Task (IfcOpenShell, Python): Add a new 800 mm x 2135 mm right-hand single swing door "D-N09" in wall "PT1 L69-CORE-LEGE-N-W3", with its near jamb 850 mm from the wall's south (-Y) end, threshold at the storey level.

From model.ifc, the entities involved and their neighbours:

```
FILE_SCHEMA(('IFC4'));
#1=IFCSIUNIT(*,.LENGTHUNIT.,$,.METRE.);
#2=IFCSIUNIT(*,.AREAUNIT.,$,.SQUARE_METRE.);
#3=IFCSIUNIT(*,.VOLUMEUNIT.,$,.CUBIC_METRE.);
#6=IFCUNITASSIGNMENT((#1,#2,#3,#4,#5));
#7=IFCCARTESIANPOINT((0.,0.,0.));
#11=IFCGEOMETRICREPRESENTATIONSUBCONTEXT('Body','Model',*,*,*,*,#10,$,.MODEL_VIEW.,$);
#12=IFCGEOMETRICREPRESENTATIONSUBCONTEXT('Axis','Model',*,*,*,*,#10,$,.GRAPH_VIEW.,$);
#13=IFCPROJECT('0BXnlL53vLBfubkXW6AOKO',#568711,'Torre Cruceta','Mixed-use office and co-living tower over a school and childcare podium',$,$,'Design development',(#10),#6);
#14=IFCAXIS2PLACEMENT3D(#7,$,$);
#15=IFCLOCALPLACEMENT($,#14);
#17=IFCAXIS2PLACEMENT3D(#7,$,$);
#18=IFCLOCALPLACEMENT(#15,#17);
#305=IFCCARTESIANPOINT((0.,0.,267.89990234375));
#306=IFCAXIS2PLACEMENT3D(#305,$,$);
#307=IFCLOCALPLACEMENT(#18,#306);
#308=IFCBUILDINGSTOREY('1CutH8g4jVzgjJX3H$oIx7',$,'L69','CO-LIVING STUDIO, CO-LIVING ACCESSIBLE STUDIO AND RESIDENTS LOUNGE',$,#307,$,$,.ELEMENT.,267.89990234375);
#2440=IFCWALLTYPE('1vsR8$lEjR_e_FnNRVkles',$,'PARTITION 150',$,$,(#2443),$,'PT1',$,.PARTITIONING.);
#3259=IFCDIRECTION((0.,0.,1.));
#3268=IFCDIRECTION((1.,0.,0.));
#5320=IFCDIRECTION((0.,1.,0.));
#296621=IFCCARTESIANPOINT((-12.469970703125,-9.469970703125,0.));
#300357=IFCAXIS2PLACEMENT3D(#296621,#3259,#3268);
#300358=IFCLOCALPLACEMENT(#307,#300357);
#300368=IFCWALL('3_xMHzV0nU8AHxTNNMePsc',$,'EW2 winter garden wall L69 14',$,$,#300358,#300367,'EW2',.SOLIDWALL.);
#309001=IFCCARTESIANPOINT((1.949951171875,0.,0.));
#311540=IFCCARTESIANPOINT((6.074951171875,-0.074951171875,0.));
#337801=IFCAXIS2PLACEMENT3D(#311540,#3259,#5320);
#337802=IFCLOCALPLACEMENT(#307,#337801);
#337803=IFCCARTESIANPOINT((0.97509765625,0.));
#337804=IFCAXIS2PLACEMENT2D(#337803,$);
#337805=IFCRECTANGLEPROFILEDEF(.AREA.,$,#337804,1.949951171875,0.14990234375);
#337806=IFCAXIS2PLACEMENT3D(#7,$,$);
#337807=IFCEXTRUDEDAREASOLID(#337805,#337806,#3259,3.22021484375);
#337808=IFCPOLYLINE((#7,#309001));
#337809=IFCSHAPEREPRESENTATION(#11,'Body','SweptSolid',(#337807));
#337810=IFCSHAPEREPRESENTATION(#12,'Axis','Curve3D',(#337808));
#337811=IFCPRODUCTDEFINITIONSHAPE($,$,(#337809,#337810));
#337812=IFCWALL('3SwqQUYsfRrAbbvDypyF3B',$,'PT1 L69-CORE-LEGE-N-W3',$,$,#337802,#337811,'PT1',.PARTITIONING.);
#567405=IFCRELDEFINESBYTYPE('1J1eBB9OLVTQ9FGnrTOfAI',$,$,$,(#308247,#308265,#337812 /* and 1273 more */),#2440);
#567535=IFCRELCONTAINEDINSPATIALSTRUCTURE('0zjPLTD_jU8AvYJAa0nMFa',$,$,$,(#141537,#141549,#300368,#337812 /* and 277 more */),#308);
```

```python
import numpy as np
import ifcopenshell
import ifcopenshell.api.feature
import ifcopenshell.api.geometry
import ifcopenshell.api.root
import ifcopenshell.api.spatial
import ifcopenshell.geom
import ifcopenshell.util.element
import ifcopenshell.util.placement
import ifcopenshell.util.representation
import ifcopenshell.util.shape
import ifcopenshell.util.unit

model = ifcopenshell.open("model.ifc")
unit_scale = ifcopenshell.util.unit.calculate_unit_scale(model)
settings = ifcopenshell.geom.settings()


def volume(element):
    """Net volume in cubic metres, openings subtracted."""
    shape = ifcopenshell.geom.create_shape(settings, element)
    return ifcopenshell.util.shape.get_volume(shape.geometry)


wall = model.by_guid("3SwqQUYsfRrAbbvDypyF3B")
storey = ifcopenshell.util.element.get_container(wall, ifc_class="IfcBuildingStorey")
context = ifcopenshell.util.representation.get_context(model, "Model", "Body", "MODEL_VIEW")
before = volume(wall)

width, height, from_end, sill = 0.8, 2.135, 0.85, 0.0  # metres

# The wall runs along its own X axis, and the end named is its -X end.
wall_shape = ifcopenshell.geom.create_shape(settings, wall)
x, y, z = ifcopenshell.util.shape.get_vertices(wall_shape.geometry).T
start = x.min() + from_end
face, thickness = float(y.min()), float(y.max() - y.min())
wall_matrix = ifcopenshell.util.placement.get_local_placement(wall.ObjectPlacement)
level = ifcopenshell.util.placement.get_local_placement(storey.ObjectPlacement)[2, 3]


def in_wall(x, y):
    """Placement at x, y metres in the wall's axes, at sill height."""
    matrix = wall_matrix.copy()
    matrix[:, 3] = wall_matrix @ np.array([x / unit_scale, y / unit_scale, 0.0, 1.0])
    matrix[2, 3] = level + sill / unit_scale
    return matrix


# Opening: a box that overshoots both wall faces by 50 mm.
opening = ifcopenshell.api.root.create_entity(model, ifc_class="IfcOpeningElement", predefined_type="OPENING")
box = ifcopenshell.api.geometry.add_wall_representation(
    model, context=context, length=width, height=height, thickness=thickness + 0.1
)
ifcopenshell.api.geometry.assign_representation(model, product=opening, representation=box)
ifcopenshell.api.geometry.edit_object_placement(model, product=opening, matrix=in_wall(start, face - 0.05), is_si=False)
ifcopenshell.api.feature.add_feature(model, feature=opening, element=wall)

door = ifcopenshell.api.root.create_entity(model, ifc_class="IfcDoor", name="D-N09", predefined_type="DOOR")
door.OverallWidth, door.OverallHeight = width / unit_scale, height / unit_scale
door.OperationType = "SINGLE_SWING_RIGHT"
body = ifcopenshell.api.geometry.add_door_representation(
    model,
    context=context,
    overall_width=door.OverallWidth,
    overall_height=door.OverallHeight,
    operation_type="SINGLE_SWING_RIGHT",
    lining_properties={"LiningDepth": thickness / unit_scale, "ThresholdDepth": thickness / unit_scale},
)
ifcopenshell.api.geometry.assign_representation(model, product=door, representation=body)
ifcopenshell.api.spatial.assign_container(model, products=[door], relating_structure=storey)
ifcopenshell.api.feature.add_filling(model, opening=opening, element=door)

# The lining spans the wall, so the door starts at the wall face.
ifcopenshell.api.geometry.edit_object_placement(model, product=door, matrix=in_wall(start, face), is_si=False)

after = volume(wall)

print(f"wall volume {before:.3f} -> {after:.3f} m3")

model.write("model_edited.ifc")
```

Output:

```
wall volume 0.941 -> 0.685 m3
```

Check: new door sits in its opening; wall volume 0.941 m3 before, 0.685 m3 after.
